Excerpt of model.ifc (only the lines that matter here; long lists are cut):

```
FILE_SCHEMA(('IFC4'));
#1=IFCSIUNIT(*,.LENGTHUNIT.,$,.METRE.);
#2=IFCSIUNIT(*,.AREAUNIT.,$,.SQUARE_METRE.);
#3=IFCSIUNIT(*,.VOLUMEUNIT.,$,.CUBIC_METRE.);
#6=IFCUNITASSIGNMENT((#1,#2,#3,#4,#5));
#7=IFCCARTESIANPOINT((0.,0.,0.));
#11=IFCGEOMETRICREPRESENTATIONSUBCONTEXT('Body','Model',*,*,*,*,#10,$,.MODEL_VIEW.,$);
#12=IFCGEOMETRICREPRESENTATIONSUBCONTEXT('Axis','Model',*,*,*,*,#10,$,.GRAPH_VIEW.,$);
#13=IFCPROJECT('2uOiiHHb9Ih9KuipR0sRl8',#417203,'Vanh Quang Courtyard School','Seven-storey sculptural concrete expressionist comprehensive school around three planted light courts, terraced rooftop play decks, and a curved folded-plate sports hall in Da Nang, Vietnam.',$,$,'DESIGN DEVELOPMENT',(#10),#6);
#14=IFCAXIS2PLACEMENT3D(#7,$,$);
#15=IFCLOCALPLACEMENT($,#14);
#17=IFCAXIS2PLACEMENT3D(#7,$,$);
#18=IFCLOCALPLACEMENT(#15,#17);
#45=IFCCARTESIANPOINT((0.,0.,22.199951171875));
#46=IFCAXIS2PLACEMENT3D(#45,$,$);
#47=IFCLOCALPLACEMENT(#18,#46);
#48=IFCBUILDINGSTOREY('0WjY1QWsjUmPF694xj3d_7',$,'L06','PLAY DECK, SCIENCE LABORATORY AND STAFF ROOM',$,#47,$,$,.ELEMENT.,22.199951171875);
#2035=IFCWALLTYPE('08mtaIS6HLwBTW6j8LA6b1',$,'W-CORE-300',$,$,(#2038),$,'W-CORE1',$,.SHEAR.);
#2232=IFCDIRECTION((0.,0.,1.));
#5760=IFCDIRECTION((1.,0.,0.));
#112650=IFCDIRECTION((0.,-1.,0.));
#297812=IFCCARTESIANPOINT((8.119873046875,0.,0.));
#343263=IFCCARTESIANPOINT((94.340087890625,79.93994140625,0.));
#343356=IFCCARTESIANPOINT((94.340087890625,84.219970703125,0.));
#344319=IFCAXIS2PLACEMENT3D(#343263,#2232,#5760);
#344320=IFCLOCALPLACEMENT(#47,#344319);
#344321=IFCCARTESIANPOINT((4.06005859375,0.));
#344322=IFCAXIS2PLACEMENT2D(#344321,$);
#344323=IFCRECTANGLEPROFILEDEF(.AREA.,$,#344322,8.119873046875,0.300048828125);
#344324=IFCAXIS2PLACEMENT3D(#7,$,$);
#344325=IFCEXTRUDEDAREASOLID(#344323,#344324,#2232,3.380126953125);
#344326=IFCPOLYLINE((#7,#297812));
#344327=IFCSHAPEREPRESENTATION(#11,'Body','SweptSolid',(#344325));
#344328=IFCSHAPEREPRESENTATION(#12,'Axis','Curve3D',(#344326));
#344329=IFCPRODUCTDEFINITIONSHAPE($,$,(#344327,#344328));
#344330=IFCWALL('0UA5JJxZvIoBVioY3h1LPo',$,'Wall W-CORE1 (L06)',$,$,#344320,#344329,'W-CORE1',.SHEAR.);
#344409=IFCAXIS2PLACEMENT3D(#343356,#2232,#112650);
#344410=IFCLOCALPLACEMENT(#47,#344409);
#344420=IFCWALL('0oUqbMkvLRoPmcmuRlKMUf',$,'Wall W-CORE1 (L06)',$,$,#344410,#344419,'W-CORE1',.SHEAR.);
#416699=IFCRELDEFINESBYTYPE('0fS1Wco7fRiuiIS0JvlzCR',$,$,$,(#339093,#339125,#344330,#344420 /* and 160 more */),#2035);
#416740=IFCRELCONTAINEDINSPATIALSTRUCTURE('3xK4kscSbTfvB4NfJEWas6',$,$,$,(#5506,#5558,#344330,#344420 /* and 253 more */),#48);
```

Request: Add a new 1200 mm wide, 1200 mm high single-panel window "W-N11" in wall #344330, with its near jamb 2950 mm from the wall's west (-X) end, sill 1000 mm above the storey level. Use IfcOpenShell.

```python
import numpy as np
import ifcopenshell
import ifcopenshell.api.feature
import ifcopenshell.api.geometry
import ifcopenshell.api.root
import ifcopenshell.api.spatial
import ifcopenshell.geom
import ifcopenshell.util.element
import ifcopenshell.util.placement
import ifcopenshell.util.representation
import ifcopenshell.util.shape
import ifcopenshell.util.unit

model = ifcopenshell.open("model.ifc")
unit_scale = ifcopenshell.util.unit.calculate_unit_scale(model)
settings = ifcopenshell.geom.settings()


def volume(element):
    """Net volume in cubic metres, openings subtracted."""
    shape = ifcopenshell.geom.create_shape(settings, element)
    return ifcopenshell.util.shape.get_volume(shape.geometry)


wall = model.by_guid("0UA5JJxZvIoBVioY3h1LPo")
storey = ifcopenshell.util.element.get_container(wall, ifc_class="IfcBuildingStorey")
context = ifcopenshell.util.representation.get_context(model, "Model", "Body", "MODEL_VIEW")
before = volume(wall)

width, height, from_end, sill = 1.2, 1.2, 2.95, 1  # metres

# The wall runs along its own X axis, and the end named is its -X end.
wall_shape = ifcopenshell.geom.create_shape(settings, wall)
x, y, z = ifcopenshell.util.shape.get_vertices(wall_shape.geometry).T
start = x.min() + from_end
face, thickness = float(y.min()), float(y.max() - y.min())
wall_matrix = ifcopenshell.util.placement.get_local_placement(wall.ObjectPlacement)
level = ifcopenshell.util.placement.get_local_placement(storey.ObjectPlacement)[2, 3]


def in_wall(x, y):
    """Placement at x, y metres in the wall's axes, at sill height."""
    matrix = wall_matrix.copy()
    matrix[:, 3] = wall_matrix @ np.array([x / unit_scale, y / unit_scale, 0.0, 1.0])
    matrix[2, 3] = level + sill / unit_scale
    return matrix


# Opening: a box that overshoots both wall faces by 50 mm.
opening = ifcopenshell.api.root.create_entity(model, ifc_class="IfcOpeningElement", predefined_type="OPENING")
box = ifcopenshell.api.geometry.add_wall_representation(
    model, context=context, length=width, height=height, thickness=thickness + 0.1
)
ifcopenshell.api.geometry.assign_representation(model, product=opening, representation=box)
ifcopenshell.api.geometry.edit_object_placement(model, product=opening, matrix=in_wall(start, face - 0.05), is_si=False)
ifcopenshell.api.feature.add_feature(model, feature=opening, element=wall)

window = ifcopenshell.api.root.create_entity(model, ifc_class="IfcWindow", name="W-N11", predefined_type="WINDOW")
window.OverallWidth, window.OverallHeight = width / unit_scale, height / unit_scale
window.PartitioningType = "SINGLE_PANEL"
body = ifcopenshell.api.geometry.add_window_representation(
    model,
    context=context,
    overall_width=window.OverallWidth,
    overall_height=window.OverallHeight,
    partition_type="SINGLE_PANEL",
)
ifcopenshell.api.geometry.assign_representation(model, product=window, representation=body)
ifcopenshell.api.spatial.assign_container(model, products=[window], relating_structure=storey)
ifcopenshell.api.feature.add_filling(model, opening=opening, element=window)

# Centre the window in the wall's thickness.
ifcopenshell.api.geometry.edit_object_placement(model, product=window, matrix=in_wall(start, face), is_si=False)
window_shape = ifcopenshell.geom.create_shape(settings, window)
depth = ifcopenshell.util.shape.get_vertices(window_shape.geometry)[:, 1]
offset = face + thickness / 2 - (depth.min() + depth.max()) / 2
ifcopenshell.api.geometry.edit_object_placement(model, product=window, matrix=in_wall(start, offset), is_si=False)

after = volume(wall)

print(f"wall volume {before:.3f} -> {after:.3f} m3")

model.write("model_rev.ifc")
```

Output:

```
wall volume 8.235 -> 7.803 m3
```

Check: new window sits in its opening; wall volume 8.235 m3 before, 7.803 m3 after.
